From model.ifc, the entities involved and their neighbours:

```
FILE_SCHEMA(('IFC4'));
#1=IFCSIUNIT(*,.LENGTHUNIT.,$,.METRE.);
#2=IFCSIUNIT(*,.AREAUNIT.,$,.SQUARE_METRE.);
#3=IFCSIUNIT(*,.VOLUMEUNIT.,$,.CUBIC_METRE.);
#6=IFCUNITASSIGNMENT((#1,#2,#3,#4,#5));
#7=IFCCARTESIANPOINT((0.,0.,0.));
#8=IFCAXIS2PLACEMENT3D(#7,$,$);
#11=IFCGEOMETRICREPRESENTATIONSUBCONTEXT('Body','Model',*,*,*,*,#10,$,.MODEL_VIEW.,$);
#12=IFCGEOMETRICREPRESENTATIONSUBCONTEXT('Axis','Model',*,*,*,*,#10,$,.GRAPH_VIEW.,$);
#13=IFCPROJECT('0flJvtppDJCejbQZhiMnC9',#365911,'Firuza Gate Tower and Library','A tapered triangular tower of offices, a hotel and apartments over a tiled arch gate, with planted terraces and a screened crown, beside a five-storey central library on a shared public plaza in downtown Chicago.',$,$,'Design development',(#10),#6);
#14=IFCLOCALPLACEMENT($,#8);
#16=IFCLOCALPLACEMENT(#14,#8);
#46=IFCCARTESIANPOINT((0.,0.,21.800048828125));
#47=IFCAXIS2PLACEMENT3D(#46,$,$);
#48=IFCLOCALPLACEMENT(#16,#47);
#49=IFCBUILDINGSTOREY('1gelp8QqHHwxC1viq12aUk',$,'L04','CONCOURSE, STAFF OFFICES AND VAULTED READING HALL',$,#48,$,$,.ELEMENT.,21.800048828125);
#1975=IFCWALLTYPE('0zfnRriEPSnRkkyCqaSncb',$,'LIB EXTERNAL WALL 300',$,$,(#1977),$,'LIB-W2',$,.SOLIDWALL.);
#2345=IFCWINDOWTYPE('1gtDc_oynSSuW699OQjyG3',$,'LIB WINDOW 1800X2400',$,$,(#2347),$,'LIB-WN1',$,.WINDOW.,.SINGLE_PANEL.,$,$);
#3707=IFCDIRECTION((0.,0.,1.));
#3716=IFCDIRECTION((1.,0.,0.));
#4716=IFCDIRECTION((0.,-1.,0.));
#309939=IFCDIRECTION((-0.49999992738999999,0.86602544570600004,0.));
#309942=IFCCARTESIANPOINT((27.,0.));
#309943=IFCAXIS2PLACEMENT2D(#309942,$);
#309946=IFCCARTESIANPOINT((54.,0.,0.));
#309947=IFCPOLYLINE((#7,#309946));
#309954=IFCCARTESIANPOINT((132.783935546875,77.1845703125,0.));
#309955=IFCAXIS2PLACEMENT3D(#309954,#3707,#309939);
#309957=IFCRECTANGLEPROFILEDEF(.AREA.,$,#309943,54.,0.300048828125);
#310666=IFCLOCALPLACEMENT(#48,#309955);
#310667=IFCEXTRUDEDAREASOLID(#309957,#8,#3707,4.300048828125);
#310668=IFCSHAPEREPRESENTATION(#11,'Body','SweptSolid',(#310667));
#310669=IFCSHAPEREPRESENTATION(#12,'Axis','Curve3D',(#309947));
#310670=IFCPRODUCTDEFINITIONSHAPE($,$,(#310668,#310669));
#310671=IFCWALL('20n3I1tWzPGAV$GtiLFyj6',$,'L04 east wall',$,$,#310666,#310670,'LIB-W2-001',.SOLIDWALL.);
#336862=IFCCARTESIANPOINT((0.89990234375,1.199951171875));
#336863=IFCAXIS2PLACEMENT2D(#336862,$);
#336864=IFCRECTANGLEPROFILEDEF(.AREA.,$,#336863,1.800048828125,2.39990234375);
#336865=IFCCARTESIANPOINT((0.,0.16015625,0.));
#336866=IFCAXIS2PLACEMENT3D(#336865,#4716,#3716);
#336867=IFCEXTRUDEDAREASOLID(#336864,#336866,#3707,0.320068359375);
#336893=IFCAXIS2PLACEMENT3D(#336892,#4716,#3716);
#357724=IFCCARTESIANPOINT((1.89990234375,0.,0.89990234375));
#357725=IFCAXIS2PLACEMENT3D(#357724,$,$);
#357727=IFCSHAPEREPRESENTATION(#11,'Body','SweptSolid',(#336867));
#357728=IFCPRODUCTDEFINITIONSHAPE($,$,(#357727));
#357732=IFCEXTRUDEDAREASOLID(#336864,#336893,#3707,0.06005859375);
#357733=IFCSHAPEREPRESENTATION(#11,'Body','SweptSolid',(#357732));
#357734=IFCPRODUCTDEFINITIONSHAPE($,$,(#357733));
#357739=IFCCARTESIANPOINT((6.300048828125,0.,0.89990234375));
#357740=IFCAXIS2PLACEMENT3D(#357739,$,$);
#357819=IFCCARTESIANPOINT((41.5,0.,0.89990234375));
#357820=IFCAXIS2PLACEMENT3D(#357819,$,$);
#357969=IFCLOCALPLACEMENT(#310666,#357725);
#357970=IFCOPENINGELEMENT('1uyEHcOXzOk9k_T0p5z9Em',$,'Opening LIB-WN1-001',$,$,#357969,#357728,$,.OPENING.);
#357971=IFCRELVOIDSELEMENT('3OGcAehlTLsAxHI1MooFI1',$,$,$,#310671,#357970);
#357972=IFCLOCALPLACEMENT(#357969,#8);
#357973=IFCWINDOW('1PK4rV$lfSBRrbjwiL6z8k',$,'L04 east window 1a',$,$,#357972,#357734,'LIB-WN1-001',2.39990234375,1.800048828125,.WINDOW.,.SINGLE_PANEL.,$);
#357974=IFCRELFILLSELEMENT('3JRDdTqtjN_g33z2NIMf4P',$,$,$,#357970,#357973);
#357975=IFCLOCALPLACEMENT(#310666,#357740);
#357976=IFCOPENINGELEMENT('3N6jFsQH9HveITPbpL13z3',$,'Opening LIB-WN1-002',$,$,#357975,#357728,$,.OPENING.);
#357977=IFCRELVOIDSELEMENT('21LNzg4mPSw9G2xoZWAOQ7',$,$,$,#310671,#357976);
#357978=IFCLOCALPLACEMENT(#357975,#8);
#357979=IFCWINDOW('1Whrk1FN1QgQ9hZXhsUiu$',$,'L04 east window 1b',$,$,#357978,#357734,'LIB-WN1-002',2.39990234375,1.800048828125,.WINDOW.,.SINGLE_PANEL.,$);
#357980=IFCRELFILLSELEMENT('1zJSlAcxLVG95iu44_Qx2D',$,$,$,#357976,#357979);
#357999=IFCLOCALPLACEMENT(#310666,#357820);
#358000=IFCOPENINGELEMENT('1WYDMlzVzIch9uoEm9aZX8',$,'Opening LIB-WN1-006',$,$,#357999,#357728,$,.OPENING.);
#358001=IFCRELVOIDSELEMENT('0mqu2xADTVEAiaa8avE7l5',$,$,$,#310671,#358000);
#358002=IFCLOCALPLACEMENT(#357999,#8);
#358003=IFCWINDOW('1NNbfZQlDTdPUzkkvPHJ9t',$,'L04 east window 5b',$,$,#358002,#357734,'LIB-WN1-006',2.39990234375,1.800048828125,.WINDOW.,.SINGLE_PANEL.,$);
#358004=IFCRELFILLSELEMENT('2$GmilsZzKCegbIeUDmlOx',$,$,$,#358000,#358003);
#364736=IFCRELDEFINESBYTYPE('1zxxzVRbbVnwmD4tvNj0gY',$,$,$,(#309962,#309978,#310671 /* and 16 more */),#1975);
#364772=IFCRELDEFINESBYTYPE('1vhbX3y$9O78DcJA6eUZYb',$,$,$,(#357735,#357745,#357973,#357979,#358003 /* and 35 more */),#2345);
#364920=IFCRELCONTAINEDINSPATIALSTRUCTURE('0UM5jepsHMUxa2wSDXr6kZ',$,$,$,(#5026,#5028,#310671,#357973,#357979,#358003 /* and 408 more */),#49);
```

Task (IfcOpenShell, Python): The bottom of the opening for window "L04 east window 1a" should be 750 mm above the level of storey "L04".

```python
import numpy as np
import ifcopenshell
import ifcopenshell.api.geometry
import ifcopenshell.geom
import ifcopenshell.util.element
import ifcopenshell.util.placement
import ifcopenshell.util.shape
import ifcopenshell.util.unit

model = ifcopenshell.open("model.ifc")
unit_scale = ifcopenshell.util.unit.calculate_unit_scale(model)

window = model.by_guid("1PK4rV$lfSBRrbjwiL6z8k")
opening = window.FillsVoids[0].RelatingOpeningElement
storey = ifcopenshell.util.element.get_container(window, ifc_class="IfcBuildingStorey")
level = ifcopenshell.util.placement.get_local_placement(storey.ObjectPlacement)[2, 3]

# The opening's origin need not be at the sill, so measure its lowest point.
shape = ifcopenshell.geom.create_shape(ifcopenshell.geom.settings(), opening)
bottom = ifcopenshell.util.shape.get_shape_bottom_elevation(shape, shape.geometry) / unit_scale
dz = level + 0.75 / unit_scale - bottom

shift = np.array([0.0, 0.0, dz])
# The window is placed relative to its opening, so it follows when the opening moves.
matrix = ifcopenshell.util.placement.get_local_placement(opening.ObjectPlacement)
matrix[:3, 3] += shift
ifcopenshell.api.geometry.edit_object_placement(
    model, product=opening, matrix=matrix, is_si=False, should_transform_children=True
)

print(f"moved by {dz * unit_scale:+.3f} m")

model.write("model_updated.ifc")
```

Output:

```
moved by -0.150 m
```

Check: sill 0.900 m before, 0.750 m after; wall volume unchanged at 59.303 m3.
